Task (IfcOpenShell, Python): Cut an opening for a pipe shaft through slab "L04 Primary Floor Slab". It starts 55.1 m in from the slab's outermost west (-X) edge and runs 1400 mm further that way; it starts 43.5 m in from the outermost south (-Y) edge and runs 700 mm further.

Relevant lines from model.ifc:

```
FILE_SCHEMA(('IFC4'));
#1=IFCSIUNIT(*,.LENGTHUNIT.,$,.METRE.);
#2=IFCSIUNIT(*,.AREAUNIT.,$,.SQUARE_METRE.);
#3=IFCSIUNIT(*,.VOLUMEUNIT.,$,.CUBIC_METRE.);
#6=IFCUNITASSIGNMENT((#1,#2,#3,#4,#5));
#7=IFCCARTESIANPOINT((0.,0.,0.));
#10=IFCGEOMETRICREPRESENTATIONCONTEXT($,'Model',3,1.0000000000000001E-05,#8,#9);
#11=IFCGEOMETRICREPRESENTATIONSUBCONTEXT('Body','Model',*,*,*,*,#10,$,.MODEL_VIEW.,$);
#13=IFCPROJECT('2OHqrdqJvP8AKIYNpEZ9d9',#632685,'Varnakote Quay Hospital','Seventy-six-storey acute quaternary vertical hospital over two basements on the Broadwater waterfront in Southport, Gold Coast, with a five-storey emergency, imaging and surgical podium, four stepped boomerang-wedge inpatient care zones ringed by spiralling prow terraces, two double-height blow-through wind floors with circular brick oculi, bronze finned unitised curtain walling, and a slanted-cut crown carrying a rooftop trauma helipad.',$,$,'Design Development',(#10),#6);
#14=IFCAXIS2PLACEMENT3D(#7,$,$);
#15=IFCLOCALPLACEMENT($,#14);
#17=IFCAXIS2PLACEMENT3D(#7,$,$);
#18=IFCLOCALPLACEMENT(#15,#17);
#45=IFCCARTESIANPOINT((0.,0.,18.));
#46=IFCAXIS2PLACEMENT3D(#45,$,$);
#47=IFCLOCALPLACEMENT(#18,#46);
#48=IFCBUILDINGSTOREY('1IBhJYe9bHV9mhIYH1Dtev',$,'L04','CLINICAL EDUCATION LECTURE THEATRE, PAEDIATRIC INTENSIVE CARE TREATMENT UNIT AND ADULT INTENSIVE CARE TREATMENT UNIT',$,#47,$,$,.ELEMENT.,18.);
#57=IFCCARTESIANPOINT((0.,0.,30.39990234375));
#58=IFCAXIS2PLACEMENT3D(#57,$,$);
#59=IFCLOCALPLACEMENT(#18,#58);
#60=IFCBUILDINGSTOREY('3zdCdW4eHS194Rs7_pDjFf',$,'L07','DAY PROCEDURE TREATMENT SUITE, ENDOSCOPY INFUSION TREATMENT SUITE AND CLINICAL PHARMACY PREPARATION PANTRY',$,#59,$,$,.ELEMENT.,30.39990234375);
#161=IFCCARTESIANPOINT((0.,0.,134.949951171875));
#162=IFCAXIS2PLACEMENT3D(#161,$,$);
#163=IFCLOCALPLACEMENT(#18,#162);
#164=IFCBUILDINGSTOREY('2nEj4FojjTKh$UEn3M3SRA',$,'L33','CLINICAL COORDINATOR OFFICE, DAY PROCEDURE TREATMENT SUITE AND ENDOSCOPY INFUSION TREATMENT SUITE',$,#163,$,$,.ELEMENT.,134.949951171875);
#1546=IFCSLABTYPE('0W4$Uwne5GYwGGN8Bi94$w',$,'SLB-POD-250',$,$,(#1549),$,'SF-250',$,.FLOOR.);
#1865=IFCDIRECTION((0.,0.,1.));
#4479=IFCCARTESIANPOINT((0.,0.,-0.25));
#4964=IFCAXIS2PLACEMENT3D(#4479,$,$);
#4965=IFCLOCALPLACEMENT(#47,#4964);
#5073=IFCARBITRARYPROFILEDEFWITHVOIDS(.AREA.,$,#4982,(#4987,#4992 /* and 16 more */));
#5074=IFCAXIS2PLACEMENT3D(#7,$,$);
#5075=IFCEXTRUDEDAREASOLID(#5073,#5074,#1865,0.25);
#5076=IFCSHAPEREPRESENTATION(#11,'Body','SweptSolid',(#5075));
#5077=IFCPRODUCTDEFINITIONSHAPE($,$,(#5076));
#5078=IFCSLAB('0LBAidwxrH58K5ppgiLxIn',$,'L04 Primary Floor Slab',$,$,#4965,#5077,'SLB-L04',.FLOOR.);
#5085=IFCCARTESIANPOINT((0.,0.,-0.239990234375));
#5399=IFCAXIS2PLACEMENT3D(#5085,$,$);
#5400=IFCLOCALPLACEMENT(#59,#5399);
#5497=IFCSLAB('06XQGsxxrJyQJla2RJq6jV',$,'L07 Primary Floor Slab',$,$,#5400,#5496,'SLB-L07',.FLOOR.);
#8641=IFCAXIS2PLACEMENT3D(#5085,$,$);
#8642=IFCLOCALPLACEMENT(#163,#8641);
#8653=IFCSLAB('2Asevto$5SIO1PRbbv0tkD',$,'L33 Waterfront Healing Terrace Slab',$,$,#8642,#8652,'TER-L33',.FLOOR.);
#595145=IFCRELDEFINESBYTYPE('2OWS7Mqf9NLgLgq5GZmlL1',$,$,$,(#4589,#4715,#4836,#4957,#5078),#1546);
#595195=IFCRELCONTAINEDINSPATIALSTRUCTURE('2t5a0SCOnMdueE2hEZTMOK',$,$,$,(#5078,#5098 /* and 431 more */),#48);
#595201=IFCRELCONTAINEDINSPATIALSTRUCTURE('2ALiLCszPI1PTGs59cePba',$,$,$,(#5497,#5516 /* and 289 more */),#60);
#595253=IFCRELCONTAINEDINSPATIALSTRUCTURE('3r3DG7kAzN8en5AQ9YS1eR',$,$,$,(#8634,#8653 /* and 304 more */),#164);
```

```python
import numpy as np
import ifcopenshell
import ifcopenshell.api.feature
import ifcopenshell.api.geometry
import ifcopenshell.api.root
import ifcopenshell.geom
import ifcopenshell.util.placement
import ifcopenshell.util.representation
import ifcopenshell.util.shape
import ifcopenshell.util.unit

model = ifcopenshell.open("model.ifc")
unit_scale = ifcopenshell.util.unit.calculate_unit_scale(model)
settings = ifcopenshell.geom.settings()


def volume(element):
    """Net volume in cubic metres, openings subtracted."""
    shape = ifcopenshell.geom.create_shape(settings, element)
    return ifcopenshell.util.shape.get_volume(shape.geometry)


slab = model.by_guid("0LBAidwxrH58K5ppgiLxIn")
before = volume(slab)

# Extent in the slab's own axes, in metres. The edges named are its -X and -Y sides.
slab_shape = ifcopenshell.geom.create_shape(settings, slab)
vertices = ifcopenshell.util.shape.get_vertices(slab_shape.geometry)
x_min, y_min, bottom = vertices.min(axis=0)
top = vertices[:, 2].max()

opening = ifcopenshell.api.root.create_entity(model, ifc_class="IfcOpeningElement", name="Pipe shaft opening", predefined_type="OPENING")
context = ifcopenshell.util.representation.get_context(model, "Model", "Body", "MODEL_VIEW")
width, depth = 1.4, 0.7
outline = [(0.0, 0.0), (width, 0.0), (width, depth), (0.0, depth), (0.0, 0.0)]
# Overshoot both faces by 50 mm so the cut is clean.
shape = ifcopenshell.api.geometry.add_slab_representation(
    model, context=context, depth=top - bottom + 0.1, polyline=outline
)
ifcopenshell.api.geometry.assign_representation(model, product=opening, representation=shape)

matrix = ifcopenshell.util.placement.get_local_placement(slab.ObjectPlacement)
matrix[:, 3] = matrix @ np.append(np.array([x_min + 55.1, y_min + 43.5, bottom - 0.05]) / unit_scale, 1.0)
ifcopenshell.api.geometry.edit_object_placement(model, product=opening, matrix=matrix, is_si=False)
ifcopenshell.api.feature.add_feature(model, feature=opening, element=slab)

after = volume(slab)

print(f"slab volume {before:.3f} -> {after:.3f} m3")

model.write("model_edited.ifc")
```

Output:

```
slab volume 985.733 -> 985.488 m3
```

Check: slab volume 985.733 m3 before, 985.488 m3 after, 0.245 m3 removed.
